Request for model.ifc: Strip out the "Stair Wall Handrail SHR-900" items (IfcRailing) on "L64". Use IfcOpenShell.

First a look at what the model holds.

```python
import ifcopenshell
import ifcopenshell.util.element

model = ifcopenshell.open("model.ifc")
print(model.schema)
storey = next(s for s in model.by_type("IfcBuildingStorey") if s.Name == "L64")
railings = [e for e in ifcopenshell.util.element.get_decomposition(storey) if e.is_a("IfcRailing")]
seen = {}
for e in railings:
    element_type = ifcopenshell.util.element.get_type(e)
    name = element_type.Name if element_type not in (None, e) else None
    seen[name] = seen.get(name, 0) + 1
for name, count in sorted(seen.items(), key=str):
    print(count, "x", name)
```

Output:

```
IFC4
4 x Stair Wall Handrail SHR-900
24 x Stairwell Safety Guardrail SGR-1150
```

```python
import ifcopenshell
import ifcopenshell.api.root
import ifcopenshell.util.element

model = ifcopenshell.open("model.ifc")

storey = next(s for s in model.by_type("IfcBuildingStorey") if s.Name == "L64")
railings = [e for e in ifcopenshell.util.element.get_decomposition(storey) if e.is_a("IfcRailing")]
targets = [e for e in railings if (t := ifcopenshell.util.element.get_type(e)) not in (None, e) and t.Name == "Stair Wall Handrail SHR-900"]

for e in targets:
    ifcopenshell.api.root.remove_product(model, product=e)
print(len(targets), "removed")

model.write("model_rev.ifc")
```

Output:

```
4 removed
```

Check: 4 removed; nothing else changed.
